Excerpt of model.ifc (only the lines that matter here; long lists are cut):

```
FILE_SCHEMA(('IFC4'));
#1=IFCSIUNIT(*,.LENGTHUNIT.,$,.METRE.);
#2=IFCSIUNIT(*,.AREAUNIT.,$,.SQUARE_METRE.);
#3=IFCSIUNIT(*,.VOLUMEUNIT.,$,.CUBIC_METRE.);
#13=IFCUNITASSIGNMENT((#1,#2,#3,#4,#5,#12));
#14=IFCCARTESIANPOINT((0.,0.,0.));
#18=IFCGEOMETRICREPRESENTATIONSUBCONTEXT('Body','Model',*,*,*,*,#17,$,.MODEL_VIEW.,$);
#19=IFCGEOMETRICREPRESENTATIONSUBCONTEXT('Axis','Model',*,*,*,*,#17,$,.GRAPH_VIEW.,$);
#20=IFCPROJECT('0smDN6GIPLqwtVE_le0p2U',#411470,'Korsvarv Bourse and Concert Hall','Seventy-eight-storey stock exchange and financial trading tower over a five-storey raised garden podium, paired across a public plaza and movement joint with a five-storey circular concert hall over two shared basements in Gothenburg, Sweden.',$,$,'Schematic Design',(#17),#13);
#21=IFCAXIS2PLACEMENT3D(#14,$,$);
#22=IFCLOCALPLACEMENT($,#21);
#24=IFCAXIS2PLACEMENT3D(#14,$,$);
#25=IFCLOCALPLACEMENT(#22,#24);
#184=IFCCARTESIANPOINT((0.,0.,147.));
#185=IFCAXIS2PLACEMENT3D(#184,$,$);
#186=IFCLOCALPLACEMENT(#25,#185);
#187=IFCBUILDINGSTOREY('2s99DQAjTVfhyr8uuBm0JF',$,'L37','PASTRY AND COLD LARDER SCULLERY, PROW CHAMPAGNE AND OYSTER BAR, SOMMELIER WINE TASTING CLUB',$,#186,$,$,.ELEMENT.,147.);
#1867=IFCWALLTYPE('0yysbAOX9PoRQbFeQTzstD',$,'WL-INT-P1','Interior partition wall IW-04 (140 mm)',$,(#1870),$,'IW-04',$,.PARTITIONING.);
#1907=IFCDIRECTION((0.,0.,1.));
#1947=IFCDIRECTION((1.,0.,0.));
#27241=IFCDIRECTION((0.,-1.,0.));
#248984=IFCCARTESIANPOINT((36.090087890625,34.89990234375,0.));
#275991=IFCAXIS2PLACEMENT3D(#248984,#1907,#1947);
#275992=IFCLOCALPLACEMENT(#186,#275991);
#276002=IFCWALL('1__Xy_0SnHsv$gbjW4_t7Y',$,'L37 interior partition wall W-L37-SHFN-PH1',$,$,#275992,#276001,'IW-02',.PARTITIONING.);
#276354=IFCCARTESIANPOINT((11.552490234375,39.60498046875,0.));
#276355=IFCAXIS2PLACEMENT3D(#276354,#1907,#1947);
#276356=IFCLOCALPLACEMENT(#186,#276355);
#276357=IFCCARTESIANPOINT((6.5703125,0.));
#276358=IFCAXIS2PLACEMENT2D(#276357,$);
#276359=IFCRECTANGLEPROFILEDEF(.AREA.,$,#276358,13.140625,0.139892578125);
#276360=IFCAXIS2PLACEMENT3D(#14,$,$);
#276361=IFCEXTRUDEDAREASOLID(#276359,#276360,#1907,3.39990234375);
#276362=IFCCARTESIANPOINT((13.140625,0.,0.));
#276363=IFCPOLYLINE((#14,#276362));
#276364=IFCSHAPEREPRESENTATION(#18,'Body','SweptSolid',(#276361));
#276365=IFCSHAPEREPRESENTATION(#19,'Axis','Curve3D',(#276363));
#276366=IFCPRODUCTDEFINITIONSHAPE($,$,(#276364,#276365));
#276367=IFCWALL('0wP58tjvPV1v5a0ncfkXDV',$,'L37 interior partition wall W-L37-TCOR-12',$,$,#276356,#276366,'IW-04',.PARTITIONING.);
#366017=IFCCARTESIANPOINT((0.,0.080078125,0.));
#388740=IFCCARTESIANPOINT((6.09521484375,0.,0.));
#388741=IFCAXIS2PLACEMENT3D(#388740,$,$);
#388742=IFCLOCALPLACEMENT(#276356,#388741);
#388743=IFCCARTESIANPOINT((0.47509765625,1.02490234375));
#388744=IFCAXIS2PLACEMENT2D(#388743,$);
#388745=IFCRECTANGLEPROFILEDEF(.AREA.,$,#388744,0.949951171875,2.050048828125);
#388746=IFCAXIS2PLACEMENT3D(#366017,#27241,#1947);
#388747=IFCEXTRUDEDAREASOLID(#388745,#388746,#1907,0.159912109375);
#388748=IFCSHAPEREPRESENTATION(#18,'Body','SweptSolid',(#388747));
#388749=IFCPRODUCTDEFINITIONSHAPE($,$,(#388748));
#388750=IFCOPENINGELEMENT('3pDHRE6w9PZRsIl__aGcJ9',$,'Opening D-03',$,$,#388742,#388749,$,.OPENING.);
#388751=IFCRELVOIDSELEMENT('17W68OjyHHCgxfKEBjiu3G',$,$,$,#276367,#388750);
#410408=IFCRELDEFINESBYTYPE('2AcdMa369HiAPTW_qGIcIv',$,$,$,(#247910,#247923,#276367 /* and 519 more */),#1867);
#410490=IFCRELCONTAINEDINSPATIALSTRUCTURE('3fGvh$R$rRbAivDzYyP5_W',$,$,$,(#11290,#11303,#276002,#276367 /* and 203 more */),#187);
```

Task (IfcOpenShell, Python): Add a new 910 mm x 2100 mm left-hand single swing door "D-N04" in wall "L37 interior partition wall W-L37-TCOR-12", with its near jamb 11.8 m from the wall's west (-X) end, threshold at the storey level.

```python
import numpy as np
import ifcopenshell
import ifcopenshell.api.feature
import ifcopenshell.api.geometry
import ifcopenshell.api.root
import ifcopenshell.api.spatial
import ifcopenshell.geom
import ifcopenshell.util.element
import ifcopenshell.util.placement
import ifcopenshell.util.representation
import ifcopenshell.util.shape
import ifcopenshell.util.unit

model = ifcopenshell.open("model.ifc")
unit_scale = ifcopenshell.util.unit.calculate_unit_scale(model)
settings = ifcopenshell.geom.settings()


def volume(element):
    """Net volume in cubic metres, openings subtracted."""
    shape = ifcopenshell.geom.create_shape(settings, element)
    return ifcopenshell.util.shape.get_volume(shape.geometry)


wall = model.by_id(276367)
storey = ifcopenshell.util.element.get_container(wall, ifc_class="IfcBuildingStorey")
context = ifcopenshell.util.representation.get_context(model, "Model", "Body", "MODEL_VIEW")
before = volume(wall)

width, height, from_end, sill = 0.91, 2.1, 11.8, 0.0  # metres

# The wall runs along its own X axis, and the end named is its -X end.
wall_shape = ifcopenshell.geom.create_shape(settings, wall)
x, y, z = ifcopenshell.util.shape.get_vertices(wall_shape.geometry).T
start = x.min() + from_end
face, thickness = float(y.min()), float(y.max() - y.min())
wall_matrix = ifcopenshell.util.placement.get_local_placement(wall.ObjectPlacement)
level = ifcopenshell.util.placement.get_local_placement(storey.ObjectPlacement)[2, 3]


def in_wall(x, y):
    """Placement at x, y metres in the wall's axes, at sill height."""
    matrix = wall_matrix.copy()
    matrix[:, 3] = wall_matrix @ np.array([x / unit_scale, y / unit_scale, 0.0, 1.0])
    matrix[2, 3] = level + sill / unit_scale
    return matrix


# Opening: a box that overshoots both wall faces by 50 mm.
opening = ifcopenshell.api.root.create_entity(model, ifc_class="IfcOpeningElement", predefined_type="OPENING")
box = ifcopenshell.api.geometry.add_wall_representation(
    model, context=context, length=width, height=height, thickness=thickness + 0.1
)
ifcopenshell.api.geometry.assign_representation(model, product=opening, representation=box)
ifcopenshell.api.geometry.edit_object_placement(model, product=opening, matrix=in_wall(start, face - 0.05), is_si=False)
ifcopenshell.api.feature.add_feature(model, feature=opening, element=wall)

door = ifcopenshell.api.root.create_entity(model, ifc_class="IfcDoor", name="D-N04", predefined_type="DOOR")
door.OverallWidth, door.OverallHeight = width / unit_scale, height / unit_scale
door.OperationType = "SINGLE_SWING_LEFT"
body = ifcopenshell.api.geometry.add_door_representation(
    model,
    context=context,
    overall_width=door.OverallWidth,
    overall_height=door.OverallHeight,
    operation_type="SINGLE_SWING_LEFT",
    lining_properties={"LiningDepth": thickness / unit_scale, "ThresholdDepth": thickness / unit_scale},
)
ifcopenshell.api.geometry.assign_representation(model, product=door, representation=body)
ifcopenshell.api.spatial.assign_container(model, products=[door], relating_structure=storey)
ifcopenshell.api.feature.add_filling(model, opening=opening, element=door)

# The lining spans the wall, so the door starts at the wall face.
ifcopenshell.api.geometry.edit_object_placement(model, product=door, matrix=in_wall(start, face), is_si=False)

after = volume(wall)

print(f"wall volume {before:.3f} -> {after:.3f} m3")

model.write("model_v2.ifc")
```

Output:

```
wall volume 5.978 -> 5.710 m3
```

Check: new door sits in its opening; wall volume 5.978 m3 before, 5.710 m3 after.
